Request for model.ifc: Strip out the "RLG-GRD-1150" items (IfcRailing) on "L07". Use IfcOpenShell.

First a look at what the model holds.

```python
import ifcopenshell
import ifcopenshell.util.element

model = ifcopenshell.open("model.ifc")
print(model.schema)
storey = next(s for s in model.by_type("IfcBuildingStorey") if s.Name == "L07")
railings = [e for e in ifcopenshell.util.element.get_decomposition(storey) if e.is_a("IfcRailing")]
seen = {}
for e in railings:
    element_type = ifcopenshell.util.element.get_type(e)
    name = element_type.Name if element_type not in (None, e) else None
    seen[name] = seen.get(name, 0) + 1
for name, count in sorted(seen.items(), key=str):
    print(count, "x", name)
```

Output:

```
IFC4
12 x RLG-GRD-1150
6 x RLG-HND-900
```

```python
import ifcopenshell
import ifcopenshell.api.root
import ifcopenshell.util.element

model = ifcopenshell.open("model.ifc")

storey = next(s for s in model.by_type("IfcBuildingStorey") if s.Name == "L07")
railings = [e for e in ifcopenshell.util.element.get_decomposition(storey) if e.is_a("IfcRailing")]
targets = [e for e in railings if (t := ifcopenshell.util.element.get_type(e)) not in (None, e) and t.Name == "RLG-GRD-1150"]

for e in targets:
    ifcopenshell.api.root.remove_product(model, product=e)
print(len(targets), "removed")

model.write("model_edited.ifc")
```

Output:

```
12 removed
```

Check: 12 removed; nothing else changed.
